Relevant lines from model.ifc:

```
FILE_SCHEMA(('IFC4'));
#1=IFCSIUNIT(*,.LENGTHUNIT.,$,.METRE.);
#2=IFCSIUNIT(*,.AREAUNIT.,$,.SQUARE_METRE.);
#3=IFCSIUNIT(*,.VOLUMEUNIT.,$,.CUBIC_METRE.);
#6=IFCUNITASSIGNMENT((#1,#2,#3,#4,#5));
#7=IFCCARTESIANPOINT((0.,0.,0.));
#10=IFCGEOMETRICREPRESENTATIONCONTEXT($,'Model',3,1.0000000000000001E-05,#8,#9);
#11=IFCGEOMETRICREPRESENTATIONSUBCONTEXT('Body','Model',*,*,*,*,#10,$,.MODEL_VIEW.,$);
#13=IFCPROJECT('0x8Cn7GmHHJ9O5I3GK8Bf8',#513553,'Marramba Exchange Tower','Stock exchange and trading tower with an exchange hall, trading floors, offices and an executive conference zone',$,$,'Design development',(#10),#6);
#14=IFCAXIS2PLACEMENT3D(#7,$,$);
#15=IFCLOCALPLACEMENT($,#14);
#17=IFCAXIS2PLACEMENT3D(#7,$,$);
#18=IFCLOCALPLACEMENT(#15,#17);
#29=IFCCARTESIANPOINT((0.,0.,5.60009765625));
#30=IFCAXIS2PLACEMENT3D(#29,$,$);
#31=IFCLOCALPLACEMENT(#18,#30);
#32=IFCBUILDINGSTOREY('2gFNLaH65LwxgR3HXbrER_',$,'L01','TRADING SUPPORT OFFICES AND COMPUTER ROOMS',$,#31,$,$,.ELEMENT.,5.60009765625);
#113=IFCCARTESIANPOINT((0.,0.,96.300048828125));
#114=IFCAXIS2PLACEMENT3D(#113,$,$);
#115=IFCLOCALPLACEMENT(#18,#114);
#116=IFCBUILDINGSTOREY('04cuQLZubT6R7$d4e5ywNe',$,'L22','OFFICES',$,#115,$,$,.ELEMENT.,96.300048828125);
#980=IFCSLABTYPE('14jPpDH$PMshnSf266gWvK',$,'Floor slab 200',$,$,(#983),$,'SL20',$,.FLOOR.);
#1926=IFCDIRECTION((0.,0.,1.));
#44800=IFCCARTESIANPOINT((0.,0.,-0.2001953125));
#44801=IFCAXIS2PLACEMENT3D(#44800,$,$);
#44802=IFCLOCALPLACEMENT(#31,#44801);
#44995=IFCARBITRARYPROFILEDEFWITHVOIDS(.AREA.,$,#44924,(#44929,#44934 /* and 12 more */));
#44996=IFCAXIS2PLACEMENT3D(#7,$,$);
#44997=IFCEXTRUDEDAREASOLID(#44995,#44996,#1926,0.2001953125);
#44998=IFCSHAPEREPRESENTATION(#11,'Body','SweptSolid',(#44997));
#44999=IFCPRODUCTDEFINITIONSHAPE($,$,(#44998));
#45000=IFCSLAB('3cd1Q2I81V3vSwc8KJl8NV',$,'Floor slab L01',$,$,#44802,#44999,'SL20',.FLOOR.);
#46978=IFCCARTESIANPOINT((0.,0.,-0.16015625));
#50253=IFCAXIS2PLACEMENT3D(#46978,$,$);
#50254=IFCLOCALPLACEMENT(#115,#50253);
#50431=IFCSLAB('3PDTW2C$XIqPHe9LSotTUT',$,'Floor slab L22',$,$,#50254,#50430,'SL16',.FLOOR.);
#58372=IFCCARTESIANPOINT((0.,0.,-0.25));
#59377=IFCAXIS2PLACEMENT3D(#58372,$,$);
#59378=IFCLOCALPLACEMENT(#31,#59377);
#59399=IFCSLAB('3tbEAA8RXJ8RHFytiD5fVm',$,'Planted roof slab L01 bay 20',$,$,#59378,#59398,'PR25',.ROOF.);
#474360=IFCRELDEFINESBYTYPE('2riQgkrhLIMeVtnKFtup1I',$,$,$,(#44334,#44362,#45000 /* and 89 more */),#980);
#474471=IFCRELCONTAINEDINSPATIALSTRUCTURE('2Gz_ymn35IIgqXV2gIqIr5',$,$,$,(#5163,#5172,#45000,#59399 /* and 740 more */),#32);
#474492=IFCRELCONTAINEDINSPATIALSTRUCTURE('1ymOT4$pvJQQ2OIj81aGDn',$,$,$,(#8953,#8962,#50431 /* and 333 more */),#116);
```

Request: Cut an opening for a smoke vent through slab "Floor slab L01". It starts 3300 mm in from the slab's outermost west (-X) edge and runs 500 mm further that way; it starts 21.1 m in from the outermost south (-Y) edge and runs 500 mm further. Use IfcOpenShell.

```python
import numpy as np
import ifcopenshell
import ifcopenshell.api.feature
import ifcopenshell.api.geometry
import ifcopenshell.api.root
import ifcopenshell.geom
import ifcopenshell.util.placement
import ifcopenshell.util.representation
import ifcopenshell.util.shape
import ifcopenshell.util.unit

model = ifcopenshell.open("model.ifc")
unit_scale = ifcopenshell.util.unit.calculate_unit_scale(model)
settings = ifcopenshell.geom.settings()


def volume(element):
    """Net volume in cubic metres, openings subtracted."""
    shape = ifcopenshell.geom.create_shape(settings, element)
    return ifcopenshell.util.shape.get_volume(shape.geometry)


slab = model.by_id(45000)
before = volume(slab)

# Extent in the slab's own axes, in metres. The edges named are its -X and -Y sides.
slab_shape = ifcopenshell.geom.create_shape(settings, slab)
vertices = ifcopenshell.util.shape.get_vertices(slab_shape.geometry)
x_min, y_min, bottom = vertices.min(axis=0)
top = vertices[:, 2].max()

opening = ifcopenshell.api.root.create_entity(model, ifc_class="IfcOpeningElement", name="Smoke vent opening", predefined_type="OPENING")
context = ifcopenshell.util.representation.get_context(model, "Model", "Body", "MODEL_VIEW")
width, depth = 0.5, 0.5
outline = [(0.0, 0.0), (width, 0.0), (width, depth), (0.0, depth), (0.0, 0.0)]
# Overshoot both faces by 50 mm so the cut is clean.
shape = ifcopenshell.api.geometry.add_slab_representation(
    model, context=context, depth=top - bottom + 0.1, polyline=outline
)
ifcopenshell.api.geometry.assign_representation(model, product=opening, representation=shape)

matrix = ifcopenshell.util.placement.get_local_placement(slab.ObjectPlacement)
matrix[:, 3] = matrix @ np.append(np.array([x_min + 3.3, y_min + 21.1, bottom - 0.05]) / unit_scale, 1.0)
ifcopenshell.api.geometry.edit_object_placement(model, product=opening, matrix=matrix, is_si=False)
ifcopenshell.api.feature.add_feature(model, feature=opening, element=slab)

after = volume(slab)

print(f"slab volume {before:.3f} -> {after:.3f} m3")

model.write("model_rev.ifc")
```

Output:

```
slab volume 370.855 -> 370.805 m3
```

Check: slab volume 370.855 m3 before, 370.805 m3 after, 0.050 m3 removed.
